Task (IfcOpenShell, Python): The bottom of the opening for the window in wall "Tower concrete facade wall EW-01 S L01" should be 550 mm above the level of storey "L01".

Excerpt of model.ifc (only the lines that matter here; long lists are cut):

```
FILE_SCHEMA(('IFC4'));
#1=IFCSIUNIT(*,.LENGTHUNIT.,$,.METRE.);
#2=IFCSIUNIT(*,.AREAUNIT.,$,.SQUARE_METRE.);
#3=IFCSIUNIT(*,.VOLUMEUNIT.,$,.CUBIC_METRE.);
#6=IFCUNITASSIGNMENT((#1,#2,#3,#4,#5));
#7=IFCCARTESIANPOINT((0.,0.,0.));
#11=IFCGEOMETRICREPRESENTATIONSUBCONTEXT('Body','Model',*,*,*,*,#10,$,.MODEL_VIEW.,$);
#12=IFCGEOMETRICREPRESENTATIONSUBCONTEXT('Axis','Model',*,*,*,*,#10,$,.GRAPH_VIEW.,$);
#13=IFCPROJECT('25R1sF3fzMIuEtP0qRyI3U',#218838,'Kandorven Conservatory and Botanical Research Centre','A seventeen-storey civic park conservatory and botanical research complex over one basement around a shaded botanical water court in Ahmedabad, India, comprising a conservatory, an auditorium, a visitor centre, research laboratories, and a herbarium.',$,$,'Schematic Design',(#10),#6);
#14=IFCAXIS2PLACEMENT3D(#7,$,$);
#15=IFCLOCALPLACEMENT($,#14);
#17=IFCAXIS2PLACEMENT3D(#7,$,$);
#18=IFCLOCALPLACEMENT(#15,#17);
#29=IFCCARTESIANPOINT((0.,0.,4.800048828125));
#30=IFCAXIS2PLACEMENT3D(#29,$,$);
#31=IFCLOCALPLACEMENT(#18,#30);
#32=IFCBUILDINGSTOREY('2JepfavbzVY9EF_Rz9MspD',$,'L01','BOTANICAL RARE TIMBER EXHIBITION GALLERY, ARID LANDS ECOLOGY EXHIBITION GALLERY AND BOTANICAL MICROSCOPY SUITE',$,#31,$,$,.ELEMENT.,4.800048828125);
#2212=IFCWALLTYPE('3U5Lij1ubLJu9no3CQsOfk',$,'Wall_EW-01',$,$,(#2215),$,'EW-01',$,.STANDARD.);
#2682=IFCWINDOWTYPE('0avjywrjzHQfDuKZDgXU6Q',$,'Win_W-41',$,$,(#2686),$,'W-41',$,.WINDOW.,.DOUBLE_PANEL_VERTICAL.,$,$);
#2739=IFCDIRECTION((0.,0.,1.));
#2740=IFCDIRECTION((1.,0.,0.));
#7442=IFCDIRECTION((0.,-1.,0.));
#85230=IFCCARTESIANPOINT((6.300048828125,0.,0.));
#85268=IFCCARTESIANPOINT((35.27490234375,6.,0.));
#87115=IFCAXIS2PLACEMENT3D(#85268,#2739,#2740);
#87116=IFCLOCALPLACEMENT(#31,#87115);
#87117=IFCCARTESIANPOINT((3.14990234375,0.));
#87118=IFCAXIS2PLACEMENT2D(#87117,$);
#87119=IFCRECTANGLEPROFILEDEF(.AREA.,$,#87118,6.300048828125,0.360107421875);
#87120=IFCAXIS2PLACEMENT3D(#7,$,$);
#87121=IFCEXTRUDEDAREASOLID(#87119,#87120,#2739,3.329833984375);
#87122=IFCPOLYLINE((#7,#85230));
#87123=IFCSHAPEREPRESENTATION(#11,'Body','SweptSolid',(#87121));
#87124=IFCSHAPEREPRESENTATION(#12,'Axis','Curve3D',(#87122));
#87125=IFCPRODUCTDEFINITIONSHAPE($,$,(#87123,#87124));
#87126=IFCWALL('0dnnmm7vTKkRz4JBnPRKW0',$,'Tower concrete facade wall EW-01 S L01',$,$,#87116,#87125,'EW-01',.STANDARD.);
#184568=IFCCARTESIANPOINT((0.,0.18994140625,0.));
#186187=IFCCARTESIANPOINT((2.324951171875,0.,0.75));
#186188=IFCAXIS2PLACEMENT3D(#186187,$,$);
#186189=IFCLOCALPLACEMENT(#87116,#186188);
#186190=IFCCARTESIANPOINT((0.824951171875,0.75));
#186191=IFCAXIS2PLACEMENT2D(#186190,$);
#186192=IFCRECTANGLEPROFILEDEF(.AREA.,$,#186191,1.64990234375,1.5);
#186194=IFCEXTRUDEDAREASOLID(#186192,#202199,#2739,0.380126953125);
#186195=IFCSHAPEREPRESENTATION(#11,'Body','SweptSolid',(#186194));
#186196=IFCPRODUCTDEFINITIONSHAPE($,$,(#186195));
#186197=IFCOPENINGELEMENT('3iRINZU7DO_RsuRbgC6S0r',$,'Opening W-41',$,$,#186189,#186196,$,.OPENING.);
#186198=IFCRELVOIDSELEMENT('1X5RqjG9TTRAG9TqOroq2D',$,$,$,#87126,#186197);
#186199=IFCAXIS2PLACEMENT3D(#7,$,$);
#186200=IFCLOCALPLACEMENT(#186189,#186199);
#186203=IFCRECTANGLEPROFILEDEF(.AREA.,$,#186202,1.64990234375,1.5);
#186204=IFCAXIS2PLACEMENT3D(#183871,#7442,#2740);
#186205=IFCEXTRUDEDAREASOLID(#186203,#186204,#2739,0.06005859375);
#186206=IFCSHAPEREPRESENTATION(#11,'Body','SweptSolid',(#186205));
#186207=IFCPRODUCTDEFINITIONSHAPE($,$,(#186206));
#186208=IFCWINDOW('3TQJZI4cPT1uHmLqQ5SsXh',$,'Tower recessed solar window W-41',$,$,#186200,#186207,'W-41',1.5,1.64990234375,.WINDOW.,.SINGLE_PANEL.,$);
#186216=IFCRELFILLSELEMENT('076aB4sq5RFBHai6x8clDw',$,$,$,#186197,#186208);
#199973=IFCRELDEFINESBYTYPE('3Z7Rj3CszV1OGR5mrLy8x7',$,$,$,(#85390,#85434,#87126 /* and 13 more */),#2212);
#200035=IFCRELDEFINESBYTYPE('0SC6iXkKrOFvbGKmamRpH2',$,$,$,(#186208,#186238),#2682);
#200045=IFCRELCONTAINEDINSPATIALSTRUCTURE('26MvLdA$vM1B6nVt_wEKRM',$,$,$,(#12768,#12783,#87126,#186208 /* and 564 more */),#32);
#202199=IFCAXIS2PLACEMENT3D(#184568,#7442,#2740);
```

```python
import numpy as np
import ifcopenshell
import ifcopenshell.api.geometry
import ifcopenshell.geom
import ifcopenshell.util.element
import ifcopenshell.util.placement
import ifcopenshell.util.shape
import ifcopenshell.util.unit

model = ifcopenshell.open("model.ifc")
unit_scale = ifcopenshell.util.unit.calculate_unit_scale(model)

window = model.by_guid("3TQJZI4cPT1uHmLqQ5SsXh")
opening = window.FillsVoids[0].RelatingOpeningElement
storey = ifcopenshell.util.element.get_container(window, ifc_class="IfcBuildingStorey")
level = ifcopenshell.util.placement.get_local_placement(storey.ObjectPlacement)[2, 3]

# The opening's origin need not be at the sill, so measure its lowest point.
shape = ifcopenshell.geom.create_shape(ifcopenshell.geom.settings(), opening)
bottom = ifcopenshell.util.shape.get_shape_bottom_elevation(shape, shape.geometry) / unit_scale
dz = level + 0.55 / unit_scale - bottom

shift = np.array([0.0, 0.0, dz])
# The window is placed relative to its opening, so it follows when the opening moves.
matrix = ifcopenshell.util.placement.get_local_placement(opening.ObjectPlacement)
matrix[:3, 3] += shift
ifcopenshell.api.geometry.edit_object_placement(
    model, product=opening, matrix=matrix, is_si=False, should_transform_children=True
)

print(f"moved by {dz * unit_scale:+.3f} m")

model.write("model_v2.ifc")
```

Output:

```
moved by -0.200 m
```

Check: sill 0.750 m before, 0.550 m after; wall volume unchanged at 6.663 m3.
